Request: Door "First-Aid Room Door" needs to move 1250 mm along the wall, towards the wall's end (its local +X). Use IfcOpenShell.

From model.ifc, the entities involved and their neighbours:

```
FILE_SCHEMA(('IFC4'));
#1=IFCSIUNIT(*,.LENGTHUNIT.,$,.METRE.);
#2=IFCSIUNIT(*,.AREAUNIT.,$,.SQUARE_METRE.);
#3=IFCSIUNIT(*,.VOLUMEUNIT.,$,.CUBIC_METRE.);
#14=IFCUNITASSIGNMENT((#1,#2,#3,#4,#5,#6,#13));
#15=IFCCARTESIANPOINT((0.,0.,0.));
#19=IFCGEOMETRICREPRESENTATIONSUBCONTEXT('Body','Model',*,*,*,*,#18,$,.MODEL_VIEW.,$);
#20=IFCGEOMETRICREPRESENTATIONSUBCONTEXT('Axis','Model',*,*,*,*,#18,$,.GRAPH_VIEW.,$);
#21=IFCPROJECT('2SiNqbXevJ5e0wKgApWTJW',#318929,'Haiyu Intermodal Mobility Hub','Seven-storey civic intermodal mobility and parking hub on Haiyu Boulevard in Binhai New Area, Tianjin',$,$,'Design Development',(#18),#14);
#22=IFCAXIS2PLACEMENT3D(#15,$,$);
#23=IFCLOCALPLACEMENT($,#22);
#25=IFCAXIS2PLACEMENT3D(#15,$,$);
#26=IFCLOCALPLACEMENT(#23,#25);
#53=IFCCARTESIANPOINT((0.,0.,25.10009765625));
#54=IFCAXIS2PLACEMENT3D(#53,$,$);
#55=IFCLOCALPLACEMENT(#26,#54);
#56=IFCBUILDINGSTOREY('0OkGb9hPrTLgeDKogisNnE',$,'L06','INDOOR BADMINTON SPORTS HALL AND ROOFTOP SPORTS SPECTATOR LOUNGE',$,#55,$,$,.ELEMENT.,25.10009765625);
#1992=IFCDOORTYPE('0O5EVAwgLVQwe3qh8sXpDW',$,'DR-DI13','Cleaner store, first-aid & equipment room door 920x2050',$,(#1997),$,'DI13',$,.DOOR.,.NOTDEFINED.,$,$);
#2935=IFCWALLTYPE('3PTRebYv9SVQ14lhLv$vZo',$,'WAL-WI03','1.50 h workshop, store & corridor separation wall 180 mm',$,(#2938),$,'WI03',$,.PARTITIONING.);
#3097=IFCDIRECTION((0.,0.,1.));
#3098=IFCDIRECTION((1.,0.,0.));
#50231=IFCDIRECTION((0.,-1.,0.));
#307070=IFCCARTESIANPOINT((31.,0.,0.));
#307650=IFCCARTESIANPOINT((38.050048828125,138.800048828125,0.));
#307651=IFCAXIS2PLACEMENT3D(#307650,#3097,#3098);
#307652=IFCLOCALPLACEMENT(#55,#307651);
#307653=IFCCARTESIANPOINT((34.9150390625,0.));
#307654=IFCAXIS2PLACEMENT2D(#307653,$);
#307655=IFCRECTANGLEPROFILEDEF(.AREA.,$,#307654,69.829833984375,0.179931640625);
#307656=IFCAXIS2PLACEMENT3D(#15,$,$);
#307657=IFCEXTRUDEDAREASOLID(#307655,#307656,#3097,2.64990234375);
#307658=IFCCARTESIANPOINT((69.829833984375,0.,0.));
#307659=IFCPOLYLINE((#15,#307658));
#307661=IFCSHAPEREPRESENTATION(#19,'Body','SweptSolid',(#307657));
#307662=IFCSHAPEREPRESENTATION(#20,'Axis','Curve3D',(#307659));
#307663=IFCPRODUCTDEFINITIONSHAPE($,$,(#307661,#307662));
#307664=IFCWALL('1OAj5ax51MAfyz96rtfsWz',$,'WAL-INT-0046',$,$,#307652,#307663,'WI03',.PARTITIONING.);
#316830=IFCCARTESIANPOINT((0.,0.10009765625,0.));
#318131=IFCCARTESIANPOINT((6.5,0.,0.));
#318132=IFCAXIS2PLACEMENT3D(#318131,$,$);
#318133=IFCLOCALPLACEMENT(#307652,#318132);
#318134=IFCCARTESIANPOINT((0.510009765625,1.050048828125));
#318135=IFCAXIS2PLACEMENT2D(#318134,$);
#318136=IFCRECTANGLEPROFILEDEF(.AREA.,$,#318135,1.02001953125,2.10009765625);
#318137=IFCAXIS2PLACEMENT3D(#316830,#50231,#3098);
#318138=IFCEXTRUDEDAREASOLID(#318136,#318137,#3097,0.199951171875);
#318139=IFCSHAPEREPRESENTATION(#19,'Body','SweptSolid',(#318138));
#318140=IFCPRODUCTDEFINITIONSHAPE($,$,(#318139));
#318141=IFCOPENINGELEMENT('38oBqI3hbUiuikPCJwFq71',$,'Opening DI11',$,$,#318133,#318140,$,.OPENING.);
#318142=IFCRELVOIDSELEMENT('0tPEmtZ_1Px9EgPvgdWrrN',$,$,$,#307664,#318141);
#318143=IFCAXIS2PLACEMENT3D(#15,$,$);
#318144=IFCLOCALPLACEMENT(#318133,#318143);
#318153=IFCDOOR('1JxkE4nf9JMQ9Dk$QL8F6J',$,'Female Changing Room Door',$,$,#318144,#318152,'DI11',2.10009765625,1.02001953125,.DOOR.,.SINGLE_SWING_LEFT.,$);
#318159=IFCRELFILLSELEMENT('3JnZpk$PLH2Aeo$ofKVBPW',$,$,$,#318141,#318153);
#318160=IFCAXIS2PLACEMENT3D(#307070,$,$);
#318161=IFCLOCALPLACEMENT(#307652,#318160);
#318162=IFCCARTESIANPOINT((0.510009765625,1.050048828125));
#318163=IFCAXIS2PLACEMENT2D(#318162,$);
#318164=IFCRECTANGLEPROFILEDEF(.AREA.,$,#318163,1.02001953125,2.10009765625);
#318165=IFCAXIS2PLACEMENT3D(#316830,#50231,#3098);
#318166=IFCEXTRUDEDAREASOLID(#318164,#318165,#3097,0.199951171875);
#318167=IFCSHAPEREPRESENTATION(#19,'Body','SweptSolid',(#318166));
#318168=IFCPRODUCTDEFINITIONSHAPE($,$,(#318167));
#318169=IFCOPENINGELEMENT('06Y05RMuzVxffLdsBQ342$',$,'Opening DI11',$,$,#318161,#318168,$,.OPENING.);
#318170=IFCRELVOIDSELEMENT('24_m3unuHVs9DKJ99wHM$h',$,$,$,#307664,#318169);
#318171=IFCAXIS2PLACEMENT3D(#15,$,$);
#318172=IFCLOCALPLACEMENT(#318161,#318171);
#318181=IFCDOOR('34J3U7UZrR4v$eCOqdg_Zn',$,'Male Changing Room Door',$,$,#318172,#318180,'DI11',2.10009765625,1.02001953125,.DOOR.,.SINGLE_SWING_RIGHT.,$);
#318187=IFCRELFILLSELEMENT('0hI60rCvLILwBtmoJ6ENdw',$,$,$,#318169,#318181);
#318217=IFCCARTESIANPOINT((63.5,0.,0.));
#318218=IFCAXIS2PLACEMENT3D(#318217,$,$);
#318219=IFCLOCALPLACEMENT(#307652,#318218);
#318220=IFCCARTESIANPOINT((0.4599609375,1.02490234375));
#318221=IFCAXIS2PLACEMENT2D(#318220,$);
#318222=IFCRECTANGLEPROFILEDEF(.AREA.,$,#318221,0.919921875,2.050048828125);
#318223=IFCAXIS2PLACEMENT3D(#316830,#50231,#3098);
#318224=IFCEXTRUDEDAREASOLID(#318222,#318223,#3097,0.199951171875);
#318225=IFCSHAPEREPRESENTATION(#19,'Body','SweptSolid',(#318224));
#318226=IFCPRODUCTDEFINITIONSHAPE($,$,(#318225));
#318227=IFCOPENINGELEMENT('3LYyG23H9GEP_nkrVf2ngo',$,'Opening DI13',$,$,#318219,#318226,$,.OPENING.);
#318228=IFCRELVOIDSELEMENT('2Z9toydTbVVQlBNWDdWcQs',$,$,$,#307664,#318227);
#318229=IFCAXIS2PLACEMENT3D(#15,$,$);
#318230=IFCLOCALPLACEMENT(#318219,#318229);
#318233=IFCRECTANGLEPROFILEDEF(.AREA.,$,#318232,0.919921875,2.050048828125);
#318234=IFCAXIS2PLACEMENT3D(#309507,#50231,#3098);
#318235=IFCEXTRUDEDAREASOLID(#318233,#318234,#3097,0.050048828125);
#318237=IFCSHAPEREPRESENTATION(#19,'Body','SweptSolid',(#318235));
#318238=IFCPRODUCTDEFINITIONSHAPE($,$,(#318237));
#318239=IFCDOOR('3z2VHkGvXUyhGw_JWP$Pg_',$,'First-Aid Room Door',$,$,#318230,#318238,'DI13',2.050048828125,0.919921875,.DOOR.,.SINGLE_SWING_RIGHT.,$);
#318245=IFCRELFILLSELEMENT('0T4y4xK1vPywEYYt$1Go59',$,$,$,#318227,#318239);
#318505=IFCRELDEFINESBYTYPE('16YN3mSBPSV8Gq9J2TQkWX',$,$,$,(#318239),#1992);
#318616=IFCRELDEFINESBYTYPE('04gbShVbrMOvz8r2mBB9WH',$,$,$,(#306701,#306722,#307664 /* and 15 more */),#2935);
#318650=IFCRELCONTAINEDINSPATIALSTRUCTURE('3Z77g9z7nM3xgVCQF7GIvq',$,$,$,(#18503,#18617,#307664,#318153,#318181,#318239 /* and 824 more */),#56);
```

```python
import ifcopenshell
import ifcopenshell.api.geometry
import ifcopenshell.util.placement

model = ifcopenshell.open("model.ifc")

door = model.by_guid("3z2VHkGvXUyhGw_JWP$Pg_")
opening = door.FillsVoids[0].RelatingOpeningElement
wall = opening.VoidsElements[0].RelatingBuildingElement

wall_matrix = ifcopenshell.util.placement.get_local_placement(wall.ObjectPlacement)
shift = wall_matrix[:3, 0] * 1.25
before = ifcopenshell.util.placement.get_local_placement(door.ObjectPlacement)[:3, 3].copy()

# The door is placed relative to its opening, so it follows when the opening moves.
matrix = ifcopenshell.util.placement.get_local_placement(opening.ObjectPlacement)
matrix[:3, 3] += shift
ifcopenshell.api.geometry.edit_object_placement(
    model, product=opening, matrix=matrix, is_si=False, should_transform_children=True
)

after = ifcopenshell.util.placement.get_local_placement(door.ObjectPlacement)[:3, 3]
print("door moved by", (after - before).round(3) + 0.0)

model.write("model_edited.ifc")
```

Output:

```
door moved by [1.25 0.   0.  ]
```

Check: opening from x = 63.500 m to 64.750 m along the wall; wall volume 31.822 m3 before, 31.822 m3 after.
